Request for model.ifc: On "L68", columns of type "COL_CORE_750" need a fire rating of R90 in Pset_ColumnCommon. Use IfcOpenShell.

First a look at what the model holds.

```python
import ifcopenshell
import ifcopenshell.util.element

model = ifcopenshell.open("model.ifc")
print(model.schema)
storey = next(s for s in model.by_type("IfcBuildingStorey") if s.Name == "L68")
columns = [e for e in ifcopenshell.util.element.get_decomposition(storey) if e.is_a("IfcColumn")]
seen = {}
for e in columns:
    element_type = ifcopenshell.util.element.get_type(e)
    key = (element_type.Name if element_type != e and element_type else None, ifcopenshell.util.element.get_pset(e, "Pset_ColumnCommon", "FireRating"))
    seen[key] = seen.get(key, 0) + 1
for (name, value), count in sorted(seen.items(), key=str):
    print(count, "x", name, "|", value)
```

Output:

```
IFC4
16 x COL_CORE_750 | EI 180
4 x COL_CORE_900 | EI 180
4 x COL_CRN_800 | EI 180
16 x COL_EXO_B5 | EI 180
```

```python
import ifcopenshell
import ifcopenshell.api.pset
import ifcopenshell.util.element

model = ifcopenshell.open("model.ifc")

storey = next(s for s in model.by_type("IfcBuildingStorey") if s.Name == "L68")
columns = [e for e in ifcopenshell.util.element.get_decomposition(storey) if e.is_a("IfcColumn")]

count = 0
for e in columns:
    element_type = ifcopenshell.util.element.get_type(e)
    if element_type in (None, e) or element_type.Name != "COL_CORE_750":
        continue
    found = ifcopenshell.util.element.get_pset(e, "Pset_ColumnCommon", should_inherit=False)
    if found:
        pset = model.by_id(found["id"])
        if len(ifcopenshell.util.element.get_elements_by_pset(pset)) > 1:
            pset = ifcopenshell.api.pset.unshare_pset(model, products=[e], pset=pset)[0]
    else:
        pset = ifcopenshell.api.pset.add_pset(model, product=e, name="Pset_ColumnCommon")
    ifcopenshell.api.pset.edit_pset(model, pset=pset, properties={"FireRating": "R90"})
    count += 1

print(count, "columns updated")

model.write("model_v2.ifc")
```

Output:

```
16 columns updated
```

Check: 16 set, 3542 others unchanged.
